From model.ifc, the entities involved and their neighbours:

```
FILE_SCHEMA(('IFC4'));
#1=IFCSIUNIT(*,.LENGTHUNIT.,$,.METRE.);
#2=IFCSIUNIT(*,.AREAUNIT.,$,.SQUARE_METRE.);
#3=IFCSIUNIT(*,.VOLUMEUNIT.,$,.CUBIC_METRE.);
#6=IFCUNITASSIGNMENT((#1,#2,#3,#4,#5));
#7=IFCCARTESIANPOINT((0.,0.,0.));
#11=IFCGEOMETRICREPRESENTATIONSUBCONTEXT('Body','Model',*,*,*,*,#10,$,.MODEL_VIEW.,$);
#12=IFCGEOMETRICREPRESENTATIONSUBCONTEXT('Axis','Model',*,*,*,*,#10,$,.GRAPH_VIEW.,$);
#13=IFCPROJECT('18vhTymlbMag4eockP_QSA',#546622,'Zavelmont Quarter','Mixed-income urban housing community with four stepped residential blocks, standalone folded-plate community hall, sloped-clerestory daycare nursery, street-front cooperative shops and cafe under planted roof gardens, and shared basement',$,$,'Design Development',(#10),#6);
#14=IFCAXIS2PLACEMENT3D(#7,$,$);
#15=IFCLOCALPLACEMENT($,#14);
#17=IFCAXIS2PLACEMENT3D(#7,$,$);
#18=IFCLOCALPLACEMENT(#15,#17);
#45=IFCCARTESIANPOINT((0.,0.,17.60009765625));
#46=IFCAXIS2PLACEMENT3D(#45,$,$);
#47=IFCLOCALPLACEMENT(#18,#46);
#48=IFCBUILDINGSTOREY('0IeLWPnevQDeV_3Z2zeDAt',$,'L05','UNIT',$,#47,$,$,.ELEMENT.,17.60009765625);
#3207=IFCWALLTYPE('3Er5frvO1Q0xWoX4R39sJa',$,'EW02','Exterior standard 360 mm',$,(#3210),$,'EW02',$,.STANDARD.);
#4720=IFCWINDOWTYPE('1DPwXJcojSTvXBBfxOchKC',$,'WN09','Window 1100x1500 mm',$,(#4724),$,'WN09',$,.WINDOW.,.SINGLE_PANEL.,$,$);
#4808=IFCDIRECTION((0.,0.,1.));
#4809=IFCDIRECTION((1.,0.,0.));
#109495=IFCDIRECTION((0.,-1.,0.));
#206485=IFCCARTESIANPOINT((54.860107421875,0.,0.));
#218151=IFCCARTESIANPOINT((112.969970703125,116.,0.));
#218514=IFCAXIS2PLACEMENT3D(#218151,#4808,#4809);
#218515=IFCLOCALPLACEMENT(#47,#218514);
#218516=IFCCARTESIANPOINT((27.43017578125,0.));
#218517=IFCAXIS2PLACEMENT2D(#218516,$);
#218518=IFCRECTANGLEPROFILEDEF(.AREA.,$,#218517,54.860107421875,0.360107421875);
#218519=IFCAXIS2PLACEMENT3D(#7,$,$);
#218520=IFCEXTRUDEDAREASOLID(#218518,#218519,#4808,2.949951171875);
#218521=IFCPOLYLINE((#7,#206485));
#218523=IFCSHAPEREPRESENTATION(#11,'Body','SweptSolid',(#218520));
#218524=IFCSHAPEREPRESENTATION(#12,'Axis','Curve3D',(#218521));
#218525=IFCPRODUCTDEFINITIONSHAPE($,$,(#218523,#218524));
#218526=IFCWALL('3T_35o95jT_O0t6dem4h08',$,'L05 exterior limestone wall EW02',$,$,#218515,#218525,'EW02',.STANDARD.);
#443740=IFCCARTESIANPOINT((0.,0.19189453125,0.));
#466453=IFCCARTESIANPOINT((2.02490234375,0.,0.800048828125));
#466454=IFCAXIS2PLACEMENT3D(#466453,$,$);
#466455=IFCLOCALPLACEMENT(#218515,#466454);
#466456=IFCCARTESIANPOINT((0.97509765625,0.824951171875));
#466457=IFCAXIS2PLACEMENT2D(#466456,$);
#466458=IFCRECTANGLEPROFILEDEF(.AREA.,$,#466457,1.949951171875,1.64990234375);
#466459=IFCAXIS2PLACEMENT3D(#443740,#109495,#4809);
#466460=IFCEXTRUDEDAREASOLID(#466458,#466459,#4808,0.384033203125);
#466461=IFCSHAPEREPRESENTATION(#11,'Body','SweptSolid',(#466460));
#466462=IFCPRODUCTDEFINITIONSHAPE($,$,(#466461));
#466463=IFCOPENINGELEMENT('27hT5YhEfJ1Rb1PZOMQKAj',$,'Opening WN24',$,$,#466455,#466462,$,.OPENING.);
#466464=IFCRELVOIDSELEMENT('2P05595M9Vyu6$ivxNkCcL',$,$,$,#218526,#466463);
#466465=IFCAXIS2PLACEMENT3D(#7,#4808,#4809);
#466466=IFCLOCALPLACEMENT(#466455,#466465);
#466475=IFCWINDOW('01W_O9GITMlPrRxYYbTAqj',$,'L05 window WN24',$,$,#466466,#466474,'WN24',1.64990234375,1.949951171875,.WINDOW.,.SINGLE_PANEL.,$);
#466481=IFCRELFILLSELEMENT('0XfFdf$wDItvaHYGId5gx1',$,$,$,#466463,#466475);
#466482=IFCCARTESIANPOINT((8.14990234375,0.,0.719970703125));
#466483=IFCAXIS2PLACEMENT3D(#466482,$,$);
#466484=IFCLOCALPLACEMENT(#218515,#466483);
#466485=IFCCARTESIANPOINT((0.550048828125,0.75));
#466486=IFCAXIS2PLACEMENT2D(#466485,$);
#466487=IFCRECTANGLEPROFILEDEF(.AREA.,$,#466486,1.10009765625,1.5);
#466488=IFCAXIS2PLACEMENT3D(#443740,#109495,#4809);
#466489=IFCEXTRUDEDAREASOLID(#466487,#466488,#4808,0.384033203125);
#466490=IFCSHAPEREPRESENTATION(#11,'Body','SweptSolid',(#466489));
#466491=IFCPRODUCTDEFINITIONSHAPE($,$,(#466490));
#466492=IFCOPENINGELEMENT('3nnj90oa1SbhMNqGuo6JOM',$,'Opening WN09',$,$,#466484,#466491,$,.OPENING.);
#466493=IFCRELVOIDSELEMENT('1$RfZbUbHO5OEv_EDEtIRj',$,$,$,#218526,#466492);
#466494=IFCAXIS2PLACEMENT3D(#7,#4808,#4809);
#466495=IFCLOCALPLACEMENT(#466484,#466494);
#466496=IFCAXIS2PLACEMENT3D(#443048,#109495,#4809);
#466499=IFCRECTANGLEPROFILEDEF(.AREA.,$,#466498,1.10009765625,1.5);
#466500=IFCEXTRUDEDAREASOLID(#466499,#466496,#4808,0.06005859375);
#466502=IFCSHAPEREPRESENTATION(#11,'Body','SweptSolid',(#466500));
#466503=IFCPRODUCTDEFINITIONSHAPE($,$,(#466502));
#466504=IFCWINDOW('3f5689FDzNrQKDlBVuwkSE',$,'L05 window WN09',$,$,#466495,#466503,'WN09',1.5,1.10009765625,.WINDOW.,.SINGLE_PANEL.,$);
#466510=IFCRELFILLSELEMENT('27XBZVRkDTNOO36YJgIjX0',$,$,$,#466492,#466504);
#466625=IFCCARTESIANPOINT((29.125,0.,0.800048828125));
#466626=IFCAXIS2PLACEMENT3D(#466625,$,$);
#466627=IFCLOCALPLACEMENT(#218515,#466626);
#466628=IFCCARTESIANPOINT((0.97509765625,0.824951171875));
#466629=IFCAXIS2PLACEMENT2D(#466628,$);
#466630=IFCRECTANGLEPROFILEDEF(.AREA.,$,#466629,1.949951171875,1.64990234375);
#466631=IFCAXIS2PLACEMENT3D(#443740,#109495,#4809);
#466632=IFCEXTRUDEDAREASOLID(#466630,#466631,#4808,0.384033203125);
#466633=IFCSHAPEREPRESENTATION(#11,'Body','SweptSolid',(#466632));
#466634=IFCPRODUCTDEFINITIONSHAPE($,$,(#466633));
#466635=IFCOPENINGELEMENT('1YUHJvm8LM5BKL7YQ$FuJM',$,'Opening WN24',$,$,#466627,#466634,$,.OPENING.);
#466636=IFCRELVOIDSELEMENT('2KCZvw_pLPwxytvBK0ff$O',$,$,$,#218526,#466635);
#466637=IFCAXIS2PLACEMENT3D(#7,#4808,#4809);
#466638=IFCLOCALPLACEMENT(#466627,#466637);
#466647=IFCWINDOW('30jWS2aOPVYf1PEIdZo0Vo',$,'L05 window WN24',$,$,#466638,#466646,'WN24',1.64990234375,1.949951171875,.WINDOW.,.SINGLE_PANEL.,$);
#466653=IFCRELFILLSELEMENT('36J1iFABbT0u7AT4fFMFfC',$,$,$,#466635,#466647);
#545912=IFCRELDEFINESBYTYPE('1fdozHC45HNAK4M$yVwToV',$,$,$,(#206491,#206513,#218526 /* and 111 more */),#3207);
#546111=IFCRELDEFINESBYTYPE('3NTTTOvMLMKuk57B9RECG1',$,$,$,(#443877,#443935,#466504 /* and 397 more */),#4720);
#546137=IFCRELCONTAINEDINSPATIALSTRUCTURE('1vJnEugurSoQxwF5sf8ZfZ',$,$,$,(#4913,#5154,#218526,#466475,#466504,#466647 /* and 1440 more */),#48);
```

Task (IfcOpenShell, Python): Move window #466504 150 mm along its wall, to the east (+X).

```python
import ifcopenshell
import ifcopenshell.api.geometry
import ifcopenshell.util.placement
import ifcopenshell.util.unit

model = ifcopenshell.open("model.ifc")
unit_scale = ifcopenshell.util.unit.calculate_unit_scale(model)

window = model.by_id(466504)
opening = window.FillsVoids[0].RelatingOpeningElement
wall = opening.VoidsElements[0].RelatingBuildingElement

wall_matrix = ifcopenshell.util.placement.get_local_placement(wall.ObjectPlacement)
shift = wall_matrix[:3, 0] * 0.15 / unit_scale
before = ifcopenshell.util.placement.get_local_placement(window.ObjectPlacement)[:3, 3].copy()

# The window is placed relative to its opening, so it follows when the opening moves.
matrix = ifcopenshell.util.placement.get_local_placement(opening.ObjectPlacement)
matrix[:3, 3] += shift
ifcopenshell.api.geometry.edit_object_placement(
    model, product=opening, matrix=matrix, is_si=False, should_transform_children=True
)

after = ifcopenshell.util.placement.get_local_placement(window.ObjectPlacement)[:3, 3]
print("window moved by", (after - before).round(3) + 0.0)

model.write("model_v2.ifc")
```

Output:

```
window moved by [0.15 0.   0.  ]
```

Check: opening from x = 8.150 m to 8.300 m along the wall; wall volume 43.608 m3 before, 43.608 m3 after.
